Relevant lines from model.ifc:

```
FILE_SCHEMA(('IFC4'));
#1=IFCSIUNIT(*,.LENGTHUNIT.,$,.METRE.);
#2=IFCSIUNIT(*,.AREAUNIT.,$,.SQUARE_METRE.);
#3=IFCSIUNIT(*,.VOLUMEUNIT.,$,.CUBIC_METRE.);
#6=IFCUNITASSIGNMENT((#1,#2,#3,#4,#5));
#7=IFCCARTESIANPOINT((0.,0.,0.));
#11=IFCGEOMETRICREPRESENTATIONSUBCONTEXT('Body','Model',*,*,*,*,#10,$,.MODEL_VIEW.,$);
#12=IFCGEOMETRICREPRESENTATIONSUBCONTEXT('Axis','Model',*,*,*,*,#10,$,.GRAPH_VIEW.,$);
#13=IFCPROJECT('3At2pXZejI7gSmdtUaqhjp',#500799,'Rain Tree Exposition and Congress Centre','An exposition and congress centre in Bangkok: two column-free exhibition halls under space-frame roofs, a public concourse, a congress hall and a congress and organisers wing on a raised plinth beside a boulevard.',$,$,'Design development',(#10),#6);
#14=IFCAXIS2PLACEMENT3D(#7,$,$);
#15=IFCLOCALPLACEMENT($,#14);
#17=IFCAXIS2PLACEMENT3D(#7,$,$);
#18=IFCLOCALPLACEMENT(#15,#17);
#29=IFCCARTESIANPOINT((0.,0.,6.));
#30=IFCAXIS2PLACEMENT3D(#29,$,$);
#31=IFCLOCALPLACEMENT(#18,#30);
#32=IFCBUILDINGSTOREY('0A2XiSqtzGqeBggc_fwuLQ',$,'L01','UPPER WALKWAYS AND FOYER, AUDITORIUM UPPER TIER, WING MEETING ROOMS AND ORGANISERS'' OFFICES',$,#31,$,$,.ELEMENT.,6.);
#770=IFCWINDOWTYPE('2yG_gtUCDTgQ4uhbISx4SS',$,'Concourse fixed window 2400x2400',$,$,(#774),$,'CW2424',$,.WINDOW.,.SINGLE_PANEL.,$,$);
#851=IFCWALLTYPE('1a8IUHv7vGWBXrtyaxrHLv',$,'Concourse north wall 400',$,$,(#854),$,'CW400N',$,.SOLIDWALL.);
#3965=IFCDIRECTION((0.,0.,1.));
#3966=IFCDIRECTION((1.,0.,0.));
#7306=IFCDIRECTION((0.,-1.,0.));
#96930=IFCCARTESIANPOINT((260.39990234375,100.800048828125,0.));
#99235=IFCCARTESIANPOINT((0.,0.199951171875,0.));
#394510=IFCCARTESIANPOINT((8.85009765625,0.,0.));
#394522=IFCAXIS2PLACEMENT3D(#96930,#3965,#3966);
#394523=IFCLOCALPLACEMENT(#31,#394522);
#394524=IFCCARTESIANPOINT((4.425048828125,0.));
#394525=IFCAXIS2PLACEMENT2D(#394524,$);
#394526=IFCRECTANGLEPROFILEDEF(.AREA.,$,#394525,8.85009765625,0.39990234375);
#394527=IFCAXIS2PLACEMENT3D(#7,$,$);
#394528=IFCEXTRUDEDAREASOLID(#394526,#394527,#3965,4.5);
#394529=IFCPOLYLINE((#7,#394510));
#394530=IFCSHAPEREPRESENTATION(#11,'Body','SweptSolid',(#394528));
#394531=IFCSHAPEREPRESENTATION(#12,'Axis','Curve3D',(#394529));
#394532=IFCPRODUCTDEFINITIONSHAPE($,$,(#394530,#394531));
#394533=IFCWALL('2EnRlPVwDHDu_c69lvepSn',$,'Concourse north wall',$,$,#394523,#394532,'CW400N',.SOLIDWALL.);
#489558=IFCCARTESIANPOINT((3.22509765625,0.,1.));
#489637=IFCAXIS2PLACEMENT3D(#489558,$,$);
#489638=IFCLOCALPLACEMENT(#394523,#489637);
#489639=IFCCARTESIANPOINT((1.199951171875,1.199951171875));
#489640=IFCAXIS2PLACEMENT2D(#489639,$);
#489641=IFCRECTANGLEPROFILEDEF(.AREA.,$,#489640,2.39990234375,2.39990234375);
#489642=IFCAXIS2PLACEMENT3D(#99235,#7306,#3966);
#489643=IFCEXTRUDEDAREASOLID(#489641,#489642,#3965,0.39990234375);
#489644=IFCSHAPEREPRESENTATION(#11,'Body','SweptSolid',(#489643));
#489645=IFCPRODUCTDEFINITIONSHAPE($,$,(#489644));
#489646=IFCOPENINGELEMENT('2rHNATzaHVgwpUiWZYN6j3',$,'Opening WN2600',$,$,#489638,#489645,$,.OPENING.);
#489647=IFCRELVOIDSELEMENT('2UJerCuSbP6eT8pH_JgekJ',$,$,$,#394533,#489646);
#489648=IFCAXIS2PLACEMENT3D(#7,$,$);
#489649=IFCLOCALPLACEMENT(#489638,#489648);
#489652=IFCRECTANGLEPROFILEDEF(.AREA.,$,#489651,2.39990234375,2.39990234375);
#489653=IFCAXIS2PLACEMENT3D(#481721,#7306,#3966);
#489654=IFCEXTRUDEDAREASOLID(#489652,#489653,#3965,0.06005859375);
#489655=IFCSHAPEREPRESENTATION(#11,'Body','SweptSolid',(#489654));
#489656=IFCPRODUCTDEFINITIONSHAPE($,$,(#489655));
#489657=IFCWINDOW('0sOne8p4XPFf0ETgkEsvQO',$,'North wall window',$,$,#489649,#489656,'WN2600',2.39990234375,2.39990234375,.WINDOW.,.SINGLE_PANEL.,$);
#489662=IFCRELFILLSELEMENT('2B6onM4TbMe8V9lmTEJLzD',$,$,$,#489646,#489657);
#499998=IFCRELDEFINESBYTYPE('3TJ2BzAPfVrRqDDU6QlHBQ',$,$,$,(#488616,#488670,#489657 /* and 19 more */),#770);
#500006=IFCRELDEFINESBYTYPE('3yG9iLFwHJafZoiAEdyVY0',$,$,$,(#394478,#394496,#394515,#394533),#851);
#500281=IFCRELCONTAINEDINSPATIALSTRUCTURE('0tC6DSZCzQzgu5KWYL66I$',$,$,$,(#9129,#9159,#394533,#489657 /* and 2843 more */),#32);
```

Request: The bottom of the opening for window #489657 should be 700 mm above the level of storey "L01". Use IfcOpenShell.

```python
import numpy as np
import ifcopenshell
import ifcopenshell.api.geometry
import ifcopenshell.geom
import ifcopenshell.util.element
import ifcopenshell.util.placement
import ifcopenshell.util.shape
import ifcopenshell.util.unit

model = ifcopenshell.open("model.ifc")
unit_scale = ifcopenshell.util.unit.calculate_unit_scale(model)

window = model.by_guid("0sOne8p4XPFf0ETgkEsvQO")
opening = window.FillsVoids[0].RelatingOpeningElement
storey = ifcopenshell.util.element.get_container(window, ifc_class="IfcBuildingStorey")
level = ifcopenshell.util.placement.get_local_placement(storey.ObjectPlacement)[2, 3]

# The opening's origin need not be at the sill, so measure its lowest point.
shape = ifcopenshell.geom.create_shape(ifcopenshell.geom.settings(), opening)
bottom = ifcopenshell.util.shape.get_shape_bottom_elevation(shape, shape.geometry) / unit_scale
dz = level + 0.7 / unit_scale - bottom

shift = np.array([0.0, 0.0, dz])
# The window is placed relative to its opening, so it follows when the opening moves.
matrix = ifcopenshell.util.placement.get_local_placement(opening.ObjectPlacement)
matrix[:3, 3] += shift
ifcopenshell.api.geometry.edit_object_placement(
    model, product=opening, matrix=matrix, is_si=False, should_transform_children=True
)

print(f"moved by {dz * unit_scale:+.3f} m")

model.write("model_v2.ifc")
```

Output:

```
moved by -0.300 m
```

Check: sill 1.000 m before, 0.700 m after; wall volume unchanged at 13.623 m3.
